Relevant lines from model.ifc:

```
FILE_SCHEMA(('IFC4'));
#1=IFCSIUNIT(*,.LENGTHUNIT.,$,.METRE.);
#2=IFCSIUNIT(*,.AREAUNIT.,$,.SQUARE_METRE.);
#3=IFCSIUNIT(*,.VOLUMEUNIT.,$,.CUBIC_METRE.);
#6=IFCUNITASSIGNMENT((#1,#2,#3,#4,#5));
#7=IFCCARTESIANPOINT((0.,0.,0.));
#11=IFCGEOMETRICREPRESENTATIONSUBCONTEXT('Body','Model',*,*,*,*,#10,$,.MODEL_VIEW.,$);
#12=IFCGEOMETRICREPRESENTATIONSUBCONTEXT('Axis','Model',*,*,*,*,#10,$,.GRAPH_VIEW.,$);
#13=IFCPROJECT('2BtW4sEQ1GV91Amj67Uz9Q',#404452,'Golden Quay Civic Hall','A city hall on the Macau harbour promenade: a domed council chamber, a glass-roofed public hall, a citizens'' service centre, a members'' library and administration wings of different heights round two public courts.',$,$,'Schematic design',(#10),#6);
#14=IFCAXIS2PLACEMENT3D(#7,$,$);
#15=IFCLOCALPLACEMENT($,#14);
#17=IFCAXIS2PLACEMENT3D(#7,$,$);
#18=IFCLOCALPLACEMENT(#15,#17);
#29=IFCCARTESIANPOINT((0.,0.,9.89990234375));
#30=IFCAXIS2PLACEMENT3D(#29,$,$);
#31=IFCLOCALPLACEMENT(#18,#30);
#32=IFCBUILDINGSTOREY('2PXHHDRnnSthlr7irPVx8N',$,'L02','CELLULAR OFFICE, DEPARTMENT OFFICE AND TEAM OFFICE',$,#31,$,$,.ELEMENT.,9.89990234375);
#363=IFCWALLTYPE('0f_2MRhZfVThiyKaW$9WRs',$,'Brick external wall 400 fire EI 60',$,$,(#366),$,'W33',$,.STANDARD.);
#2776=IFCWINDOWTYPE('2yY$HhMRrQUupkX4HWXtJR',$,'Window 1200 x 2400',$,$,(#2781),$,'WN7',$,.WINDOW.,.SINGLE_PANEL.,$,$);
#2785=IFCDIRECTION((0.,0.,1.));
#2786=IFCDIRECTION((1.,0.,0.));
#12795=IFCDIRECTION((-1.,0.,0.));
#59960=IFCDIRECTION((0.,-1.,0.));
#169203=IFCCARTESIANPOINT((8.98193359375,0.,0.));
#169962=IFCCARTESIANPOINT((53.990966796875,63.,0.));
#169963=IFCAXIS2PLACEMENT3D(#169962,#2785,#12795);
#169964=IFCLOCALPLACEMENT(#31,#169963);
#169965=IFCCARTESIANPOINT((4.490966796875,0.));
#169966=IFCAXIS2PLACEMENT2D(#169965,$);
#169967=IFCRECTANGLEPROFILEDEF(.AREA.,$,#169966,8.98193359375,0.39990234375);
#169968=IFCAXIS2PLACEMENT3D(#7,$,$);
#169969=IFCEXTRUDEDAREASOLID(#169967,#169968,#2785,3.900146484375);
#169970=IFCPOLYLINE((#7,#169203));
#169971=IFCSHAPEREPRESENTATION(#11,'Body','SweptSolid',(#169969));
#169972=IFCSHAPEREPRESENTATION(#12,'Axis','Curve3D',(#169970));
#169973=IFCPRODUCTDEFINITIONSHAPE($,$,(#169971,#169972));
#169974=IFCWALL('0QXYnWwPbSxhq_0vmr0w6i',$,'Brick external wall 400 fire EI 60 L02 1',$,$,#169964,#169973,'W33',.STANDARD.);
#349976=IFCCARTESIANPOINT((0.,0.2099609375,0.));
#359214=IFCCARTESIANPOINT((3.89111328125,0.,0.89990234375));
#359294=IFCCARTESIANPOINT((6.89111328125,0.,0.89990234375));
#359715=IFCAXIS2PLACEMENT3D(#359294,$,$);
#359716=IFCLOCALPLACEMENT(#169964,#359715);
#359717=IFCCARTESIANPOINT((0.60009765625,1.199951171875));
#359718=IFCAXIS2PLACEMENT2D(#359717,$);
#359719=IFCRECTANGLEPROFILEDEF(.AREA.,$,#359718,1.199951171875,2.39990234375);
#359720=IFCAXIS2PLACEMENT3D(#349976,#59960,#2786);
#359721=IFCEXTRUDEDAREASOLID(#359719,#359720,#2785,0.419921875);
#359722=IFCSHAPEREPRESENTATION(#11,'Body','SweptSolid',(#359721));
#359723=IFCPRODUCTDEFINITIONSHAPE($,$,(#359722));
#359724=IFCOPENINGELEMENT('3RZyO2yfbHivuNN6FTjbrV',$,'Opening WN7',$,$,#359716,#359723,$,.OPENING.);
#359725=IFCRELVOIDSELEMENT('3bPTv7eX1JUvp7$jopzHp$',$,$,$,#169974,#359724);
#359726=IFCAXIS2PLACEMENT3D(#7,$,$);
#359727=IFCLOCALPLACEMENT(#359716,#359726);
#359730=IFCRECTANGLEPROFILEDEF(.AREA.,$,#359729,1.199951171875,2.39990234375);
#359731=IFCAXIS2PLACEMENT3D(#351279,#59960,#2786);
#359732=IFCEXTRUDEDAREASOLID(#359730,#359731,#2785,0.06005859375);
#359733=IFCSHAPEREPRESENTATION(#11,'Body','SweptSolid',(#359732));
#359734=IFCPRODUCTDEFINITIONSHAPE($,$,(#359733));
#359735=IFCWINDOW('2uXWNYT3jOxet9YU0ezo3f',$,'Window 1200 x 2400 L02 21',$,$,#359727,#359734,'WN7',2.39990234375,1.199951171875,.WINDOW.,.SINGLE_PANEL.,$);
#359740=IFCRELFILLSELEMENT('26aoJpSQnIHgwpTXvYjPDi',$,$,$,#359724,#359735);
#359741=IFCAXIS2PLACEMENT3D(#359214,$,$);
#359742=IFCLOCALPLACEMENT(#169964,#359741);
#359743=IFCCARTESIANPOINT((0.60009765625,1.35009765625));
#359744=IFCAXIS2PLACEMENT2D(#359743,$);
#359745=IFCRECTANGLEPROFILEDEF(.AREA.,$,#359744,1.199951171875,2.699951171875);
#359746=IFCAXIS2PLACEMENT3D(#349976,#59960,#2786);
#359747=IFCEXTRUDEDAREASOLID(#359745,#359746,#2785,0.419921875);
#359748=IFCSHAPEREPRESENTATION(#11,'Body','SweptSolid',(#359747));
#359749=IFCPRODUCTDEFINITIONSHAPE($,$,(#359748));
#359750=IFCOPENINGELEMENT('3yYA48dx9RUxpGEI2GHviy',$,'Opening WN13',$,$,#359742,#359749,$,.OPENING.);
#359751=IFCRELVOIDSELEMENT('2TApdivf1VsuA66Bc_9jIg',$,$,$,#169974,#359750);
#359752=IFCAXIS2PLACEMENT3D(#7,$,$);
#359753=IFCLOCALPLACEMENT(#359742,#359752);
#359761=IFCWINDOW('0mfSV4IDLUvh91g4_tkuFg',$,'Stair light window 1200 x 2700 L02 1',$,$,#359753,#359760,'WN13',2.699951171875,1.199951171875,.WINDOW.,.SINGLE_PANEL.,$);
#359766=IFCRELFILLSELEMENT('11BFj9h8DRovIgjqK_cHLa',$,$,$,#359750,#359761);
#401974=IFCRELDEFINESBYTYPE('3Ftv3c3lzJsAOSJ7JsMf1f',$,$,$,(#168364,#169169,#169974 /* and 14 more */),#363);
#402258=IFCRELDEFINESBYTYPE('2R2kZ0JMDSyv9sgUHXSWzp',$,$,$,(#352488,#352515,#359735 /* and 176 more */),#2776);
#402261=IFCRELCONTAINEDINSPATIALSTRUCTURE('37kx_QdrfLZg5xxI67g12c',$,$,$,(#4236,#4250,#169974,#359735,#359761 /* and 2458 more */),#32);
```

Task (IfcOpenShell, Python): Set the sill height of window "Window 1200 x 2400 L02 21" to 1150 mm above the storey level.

```python
import numpy as np
import ifcopenshell
import ifcopenshell.api.geometry
import ifcopenshell.geom
import ifcopenshell.util.element
import ifcopenshell.util.placement
import ifcopenshell.util.shape
import ifcopenshell.util.unit

model = ifcopenshell.open("model.ifc")
unit_scale = ifcopenshell.util.unit.calculate_unit_scale(model)

window = model.by_guid("2uXWNYT3jOxet9YU0ezo3f")
opening = window.FillsVoids[0].RelatingOpeningElement
storey = ifcopenshell.util.element.get_container(window, ifc_class="IfcBuildingStorey")
level = ifcopenshell.util.placement.get_local_placement(storey.ObjectPlacement)[2, 3]

# The opening's origin need not be at the sill, so measure its lowest point.
shape = ifcopenshell.geom.create_shape(ifcopenshell.geom.settings(), opening)
bottom = ifcopenshell.util.shape.get_shape_bottom_elevation(shape, shape.geometry) / unit_scale
dz = level + 1.15 / unit_scale - bottom

shift = np.array([0.0, 0.0, dz])
# The window is placed relative to its opening, so it follows when the opening moves.
matrix = ifcopenshell.util.placement.get_local_placement(opening.ObjectPlacement)
matrix[:3, 3] += shift
ifcopenshell.api.geometry.edit_object_placement(
    model, product=opening, matrix=matrix, is_si=False, should_transform_children=True
)

print(f"moved by {dz * unit_scale:+.3f} m")

model.write("model_rev.ifc")
```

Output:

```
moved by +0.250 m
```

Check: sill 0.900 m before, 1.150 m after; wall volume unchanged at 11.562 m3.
